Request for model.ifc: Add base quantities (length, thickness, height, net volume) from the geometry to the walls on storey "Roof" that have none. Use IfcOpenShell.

First a look at what the model holds.

```python
import ifcopenshell
import ifcopenshell.util.element
import ifcopenshell.util.unit

model = ifcopenshell.open("model.ifc")
print(model.schema)
for unit_type in ("LENGTHUNIT", "AREAUNIT", "VOLUMEUNIT"):
    print(unit_type, ifcopenshell.util.unit.calculate_unit_scale(model, unit_type))
storey = next(s for s in model.by_type("IfcBuildingStorey") if s.Name == "Roof")
walls = [e for e in ifcopenshell.util.element.get_decomposition(storey) if e.is_a("IfcWall")]
for e in sorted(walls, key=lambda e: e.id()):
    print(e.id(), e.is_a(), e.Name, list(ifcopenshell.util.element.get_psets(e, qtos_only=True)), sep=" | ")
```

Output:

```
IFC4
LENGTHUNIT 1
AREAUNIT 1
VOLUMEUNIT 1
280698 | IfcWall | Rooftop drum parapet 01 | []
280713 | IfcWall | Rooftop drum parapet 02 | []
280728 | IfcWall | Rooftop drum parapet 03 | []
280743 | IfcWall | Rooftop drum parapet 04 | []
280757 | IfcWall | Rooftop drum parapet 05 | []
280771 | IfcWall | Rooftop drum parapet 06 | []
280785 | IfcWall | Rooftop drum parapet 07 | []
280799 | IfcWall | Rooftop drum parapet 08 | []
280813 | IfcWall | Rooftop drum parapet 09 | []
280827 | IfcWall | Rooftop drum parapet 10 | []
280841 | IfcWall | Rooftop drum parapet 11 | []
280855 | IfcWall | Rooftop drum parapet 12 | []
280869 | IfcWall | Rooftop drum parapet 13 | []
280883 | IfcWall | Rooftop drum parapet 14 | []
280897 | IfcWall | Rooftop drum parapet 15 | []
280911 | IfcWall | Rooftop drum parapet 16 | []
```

```python
import ifcopenshell
import ifcopenshell.api.pset
import ifcopenshell.geom
import ifcopenshell.util.element
import ifcopenshell.util.shape
import ifcopenshell.util.unit

model = ifcopenshell.open("model.ifc")
unit_scale = ifcopenshell.util.unit.calculate_unit_scale(model)
volume_scale = ifcopenshell.util.unit.calculate_unit_scale(model, "VOLUMEUNIT")
settings = ifcopenshell.geom.settings()

storey = next(s for s in model.by_type("IfcBuildingStorey") if s.Name == "Roof")
walls = [e for e in ifcopenshell.util.element.get_decomposition(storey) if e.is_a("IfcWall")]

for e in sorted(walls, key=lambda e: e.id()):
    if ifcopenshell.util.element.get_psets(e, qtos_only=True, should_inherit=False):
        continue
    # Geometry comes back in metres, in the element's own axes.
    shape = ifcopenshell.geom.create_shape(settings, e)
    values = {
        "Length": ifcopenshell.util.shape.get_x(shape.geometry) / unit_scale,
        "Width": ifcopenshell.util.shape.get_y(shape.geometry) / unit_scale,
        "Height": ifcopenshell.util.shape.get_z(shape.geometry) / unit_scale,
        "NetVolume": ifcopenshell.util.shape.get_volume(shape.geometry) / volume_scale,
    }
    qto = ifcopenshell.api.pset.add_qto(model, product=e, name="Qto_WallBaseQuantities")
    ifcopenshell.api.pset.edit_qto(model, qto=qto, properties=values)
    print(e.id(), {k: round(v, 3) for k, v in values.items()})

model.write("model-out.ifc")
```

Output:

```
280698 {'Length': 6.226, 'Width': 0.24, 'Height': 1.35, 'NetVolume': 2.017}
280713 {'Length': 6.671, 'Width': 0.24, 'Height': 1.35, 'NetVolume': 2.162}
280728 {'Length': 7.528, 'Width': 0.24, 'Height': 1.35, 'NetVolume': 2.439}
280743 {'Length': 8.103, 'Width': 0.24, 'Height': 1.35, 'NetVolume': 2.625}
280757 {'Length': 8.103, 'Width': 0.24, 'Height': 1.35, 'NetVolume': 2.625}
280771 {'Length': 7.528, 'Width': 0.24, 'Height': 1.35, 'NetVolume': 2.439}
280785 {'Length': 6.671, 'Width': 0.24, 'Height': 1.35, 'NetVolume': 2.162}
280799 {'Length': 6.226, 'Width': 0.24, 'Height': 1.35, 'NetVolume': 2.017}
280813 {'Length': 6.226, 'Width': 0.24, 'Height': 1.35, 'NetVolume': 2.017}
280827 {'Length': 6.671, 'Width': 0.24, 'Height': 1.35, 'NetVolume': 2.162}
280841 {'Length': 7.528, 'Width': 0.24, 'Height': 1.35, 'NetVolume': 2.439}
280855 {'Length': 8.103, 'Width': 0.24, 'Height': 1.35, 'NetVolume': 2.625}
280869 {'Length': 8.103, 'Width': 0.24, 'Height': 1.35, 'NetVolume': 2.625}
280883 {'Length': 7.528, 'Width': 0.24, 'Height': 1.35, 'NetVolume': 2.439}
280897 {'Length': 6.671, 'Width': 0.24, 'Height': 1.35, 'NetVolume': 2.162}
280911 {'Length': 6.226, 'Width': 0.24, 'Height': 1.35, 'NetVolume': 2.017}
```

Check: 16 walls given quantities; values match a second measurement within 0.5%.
